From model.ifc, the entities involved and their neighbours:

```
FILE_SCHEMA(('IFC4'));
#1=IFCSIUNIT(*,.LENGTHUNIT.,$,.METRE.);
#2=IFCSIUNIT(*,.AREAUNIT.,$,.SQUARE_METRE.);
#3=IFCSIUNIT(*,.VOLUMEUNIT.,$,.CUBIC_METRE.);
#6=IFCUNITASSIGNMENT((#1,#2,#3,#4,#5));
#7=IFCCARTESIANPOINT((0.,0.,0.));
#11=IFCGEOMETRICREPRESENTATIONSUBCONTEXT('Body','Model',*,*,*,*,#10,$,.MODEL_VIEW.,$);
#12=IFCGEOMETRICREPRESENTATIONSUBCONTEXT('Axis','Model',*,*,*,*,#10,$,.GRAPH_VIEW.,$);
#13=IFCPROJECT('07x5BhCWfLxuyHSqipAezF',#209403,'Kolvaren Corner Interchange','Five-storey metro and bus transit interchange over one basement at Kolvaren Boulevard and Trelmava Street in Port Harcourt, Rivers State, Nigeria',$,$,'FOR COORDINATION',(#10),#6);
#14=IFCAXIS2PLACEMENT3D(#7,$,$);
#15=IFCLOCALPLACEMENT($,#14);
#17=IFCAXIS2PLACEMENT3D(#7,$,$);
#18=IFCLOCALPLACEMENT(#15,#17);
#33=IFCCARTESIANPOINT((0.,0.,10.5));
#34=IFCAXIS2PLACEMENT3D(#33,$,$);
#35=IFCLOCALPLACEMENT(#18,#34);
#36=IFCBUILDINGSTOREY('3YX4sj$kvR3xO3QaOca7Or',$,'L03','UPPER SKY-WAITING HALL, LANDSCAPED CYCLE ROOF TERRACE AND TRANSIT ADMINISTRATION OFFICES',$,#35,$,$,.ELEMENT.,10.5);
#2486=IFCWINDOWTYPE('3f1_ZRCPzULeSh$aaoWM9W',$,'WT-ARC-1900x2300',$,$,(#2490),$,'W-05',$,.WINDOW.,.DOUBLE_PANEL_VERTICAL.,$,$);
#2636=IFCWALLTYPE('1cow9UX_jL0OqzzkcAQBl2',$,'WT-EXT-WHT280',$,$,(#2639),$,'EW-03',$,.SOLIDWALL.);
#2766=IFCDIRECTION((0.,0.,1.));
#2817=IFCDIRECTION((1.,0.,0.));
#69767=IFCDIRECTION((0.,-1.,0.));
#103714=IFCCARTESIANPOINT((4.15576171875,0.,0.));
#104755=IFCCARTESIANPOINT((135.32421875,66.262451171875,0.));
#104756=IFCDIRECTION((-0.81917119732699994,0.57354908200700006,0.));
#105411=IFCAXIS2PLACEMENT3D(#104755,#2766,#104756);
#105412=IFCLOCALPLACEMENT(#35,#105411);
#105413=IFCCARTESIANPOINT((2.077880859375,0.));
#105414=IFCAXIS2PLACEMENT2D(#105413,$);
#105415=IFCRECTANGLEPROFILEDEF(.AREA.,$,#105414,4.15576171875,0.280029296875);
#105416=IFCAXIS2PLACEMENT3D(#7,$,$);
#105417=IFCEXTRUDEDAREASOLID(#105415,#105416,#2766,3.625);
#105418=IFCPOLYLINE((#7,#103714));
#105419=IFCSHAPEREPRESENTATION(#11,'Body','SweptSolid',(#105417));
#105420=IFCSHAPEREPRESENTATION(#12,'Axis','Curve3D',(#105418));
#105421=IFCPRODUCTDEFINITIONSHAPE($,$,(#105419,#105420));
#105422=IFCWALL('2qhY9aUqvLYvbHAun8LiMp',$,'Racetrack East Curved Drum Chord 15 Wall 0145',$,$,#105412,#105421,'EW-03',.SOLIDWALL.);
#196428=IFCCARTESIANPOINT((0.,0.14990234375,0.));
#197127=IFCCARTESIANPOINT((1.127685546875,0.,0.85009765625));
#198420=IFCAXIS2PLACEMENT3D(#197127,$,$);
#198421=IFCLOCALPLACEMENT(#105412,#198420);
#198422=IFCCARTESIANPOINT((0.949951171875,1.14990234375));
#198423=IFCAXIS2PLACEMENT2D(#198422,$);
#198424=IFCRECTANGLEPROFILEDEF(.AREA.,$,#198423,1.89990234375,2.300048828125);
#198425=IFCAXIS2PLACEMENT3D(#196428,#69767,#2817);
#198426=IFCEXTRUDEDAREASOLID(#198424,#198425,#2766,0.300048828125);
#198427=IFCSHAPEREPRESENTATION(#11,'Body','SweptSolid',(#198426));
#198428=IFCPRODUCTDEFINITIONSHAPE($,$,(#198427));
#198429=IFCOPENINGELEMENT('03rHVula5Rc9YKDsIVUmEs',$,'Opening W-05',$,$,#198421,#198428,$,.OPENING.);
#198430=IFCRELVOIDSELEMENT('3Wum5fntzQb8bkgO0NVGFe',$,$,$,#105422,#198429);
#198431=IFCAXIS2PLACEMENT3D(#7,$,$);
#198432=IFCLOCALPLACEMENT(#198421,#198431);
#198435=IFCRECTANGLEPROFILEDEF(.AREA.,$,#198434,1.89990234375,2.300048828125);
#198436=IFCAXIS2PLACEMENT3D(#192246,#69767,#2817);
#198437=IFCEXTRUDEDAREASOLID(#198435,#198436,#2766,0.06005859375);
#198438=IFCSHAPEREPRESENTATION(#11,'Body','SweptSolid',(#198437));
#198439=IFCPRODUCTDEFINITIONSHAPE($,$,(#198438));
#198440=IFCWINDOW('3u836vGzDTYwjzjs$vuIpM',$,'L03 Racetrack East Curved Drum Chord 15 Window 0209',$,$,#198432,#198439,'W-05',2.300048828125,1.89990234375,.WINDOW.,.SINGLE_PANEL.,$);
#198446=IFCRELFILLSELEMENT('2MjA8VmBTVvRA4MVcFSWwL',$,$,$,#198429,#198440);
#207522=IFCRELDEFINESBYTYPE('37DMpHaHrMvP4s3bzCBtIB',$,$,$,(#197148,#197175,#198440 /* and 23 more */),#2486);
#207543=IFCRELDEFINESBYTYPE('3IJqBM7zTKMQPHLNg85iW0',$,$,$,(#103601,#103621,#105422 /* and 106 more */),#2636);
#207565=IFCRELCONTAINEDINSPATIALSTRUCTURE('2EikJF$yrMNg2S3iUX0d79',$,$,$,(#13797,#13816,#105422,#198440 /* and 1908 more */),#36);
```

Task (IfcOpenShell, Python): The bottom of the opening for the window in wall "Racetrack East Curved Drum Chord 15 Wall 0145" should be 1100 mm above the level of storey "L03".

```python
import numpy as np
import ifcopenshell
import ifcopenshell.api.geometry
import ifcopenshell.geom
import ifcopenshell.util.element
import ifcopenshell.util.placement
import ifcopenshell.util.shape
import ifcopenshell.util.unit

model = ifcopenshell.open("model.ifc")
unit_scale = ifcopenshell.util.unit.calculate_unit_scale(model)

window = model.by_guid("3u836vGzDTYwjzjs$vuIpM")
opening = window.FillsVoids[0].RelatingOpeningElement
storey = ifcopenshell.util.element.get_container(window, ifc_class="IfcBuildingStorey")
level = ifcopenshell.util.placement.get_local_placement(storey.ObjectPlacement)[2, 3]

# The opening's origin need not be at the sill, so measure its lowest point.
shape = ifcopenshell.geom.create_shape(ifcopenshell.geom.settings(), opening)
bottom = ifcopenshell.util.shape.get_shape_bottom_elevation(shape, shape.geometry) / unit_scale
dz = level + 1.1 - bottom

shift = np.array([0.0, 0.0, dz])
# The window is placed relative to its opening, so it follows when the opening moves.
matrix = ifcopenshell.util.placement.get_local_placement(opening.ObjectPlacement)
matrix[:3, 3] += shift
ifcopenshell.api.geometry.edit_object_placement(
    model, product=opening, matrix=matrix, is_si=False, should_transform_children=True
)

print(f"moved by {dz * unit_scale:+.3f} m")

model.write("model_rev.ifc")
```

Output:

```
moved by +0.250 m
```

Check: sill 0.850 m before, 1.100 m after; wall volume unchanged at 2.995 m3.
